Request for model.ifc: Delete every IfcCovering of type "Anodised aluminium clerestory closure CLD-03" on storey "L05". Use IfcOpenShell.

First a look at what the model holds.

```python
import ifcopenshell
import ifcopenshell.util.element

model = ifcopenshell.open("model.ifc")
print(model.schema)
storey = next(s for s in model.by_type("IfcBuildingStorey") if s.Name == "L05")
coverings = [e for e in ifcopenshell.util.element.get_decomposition(storey) if e.is_a("IfcCovering")]
seen = {}
for e in coverings:
    element_type = ifcopenshell.util.element.get_type(e)
    name = element_type.Name if element_type not in (None, e) else None
    seen[name] = seen.get(name, 0) + 1
for name, count in sorted(seen.items(), key=str):
    print(count, "x", name)
```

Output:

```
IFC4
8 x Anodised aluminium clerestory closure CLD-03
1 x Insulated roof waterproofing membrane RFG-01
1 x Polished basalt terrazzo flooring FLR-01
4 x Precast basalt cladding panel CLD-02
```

```python
import ifcopenshell
import ifcopenshell.api.root
import ifcopenshell.util.element

model = ifcopenshell.open("model.ifc")

storey = next(s for s in model.by_type("IfcBuildingStorey") if s.Name == "L05")
coverings = [e for e in ifcopenshell.util.element.get_decomposition(storey) if e.is_a("IfcCovering")]
targets = [e for e in coverings if (t := ifcopenshell.util.element.get_type(e)) not in (None, e) and t.Name == "Anodised aluminium clerestory closure CLD-03"]

for e in targets:
    ifcopenshell.api.root.remove_product(model, product=e)
print(len(targets), "removed")

model.write("model_rev.ifc")
```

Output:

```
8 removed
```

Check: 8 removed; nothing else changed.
